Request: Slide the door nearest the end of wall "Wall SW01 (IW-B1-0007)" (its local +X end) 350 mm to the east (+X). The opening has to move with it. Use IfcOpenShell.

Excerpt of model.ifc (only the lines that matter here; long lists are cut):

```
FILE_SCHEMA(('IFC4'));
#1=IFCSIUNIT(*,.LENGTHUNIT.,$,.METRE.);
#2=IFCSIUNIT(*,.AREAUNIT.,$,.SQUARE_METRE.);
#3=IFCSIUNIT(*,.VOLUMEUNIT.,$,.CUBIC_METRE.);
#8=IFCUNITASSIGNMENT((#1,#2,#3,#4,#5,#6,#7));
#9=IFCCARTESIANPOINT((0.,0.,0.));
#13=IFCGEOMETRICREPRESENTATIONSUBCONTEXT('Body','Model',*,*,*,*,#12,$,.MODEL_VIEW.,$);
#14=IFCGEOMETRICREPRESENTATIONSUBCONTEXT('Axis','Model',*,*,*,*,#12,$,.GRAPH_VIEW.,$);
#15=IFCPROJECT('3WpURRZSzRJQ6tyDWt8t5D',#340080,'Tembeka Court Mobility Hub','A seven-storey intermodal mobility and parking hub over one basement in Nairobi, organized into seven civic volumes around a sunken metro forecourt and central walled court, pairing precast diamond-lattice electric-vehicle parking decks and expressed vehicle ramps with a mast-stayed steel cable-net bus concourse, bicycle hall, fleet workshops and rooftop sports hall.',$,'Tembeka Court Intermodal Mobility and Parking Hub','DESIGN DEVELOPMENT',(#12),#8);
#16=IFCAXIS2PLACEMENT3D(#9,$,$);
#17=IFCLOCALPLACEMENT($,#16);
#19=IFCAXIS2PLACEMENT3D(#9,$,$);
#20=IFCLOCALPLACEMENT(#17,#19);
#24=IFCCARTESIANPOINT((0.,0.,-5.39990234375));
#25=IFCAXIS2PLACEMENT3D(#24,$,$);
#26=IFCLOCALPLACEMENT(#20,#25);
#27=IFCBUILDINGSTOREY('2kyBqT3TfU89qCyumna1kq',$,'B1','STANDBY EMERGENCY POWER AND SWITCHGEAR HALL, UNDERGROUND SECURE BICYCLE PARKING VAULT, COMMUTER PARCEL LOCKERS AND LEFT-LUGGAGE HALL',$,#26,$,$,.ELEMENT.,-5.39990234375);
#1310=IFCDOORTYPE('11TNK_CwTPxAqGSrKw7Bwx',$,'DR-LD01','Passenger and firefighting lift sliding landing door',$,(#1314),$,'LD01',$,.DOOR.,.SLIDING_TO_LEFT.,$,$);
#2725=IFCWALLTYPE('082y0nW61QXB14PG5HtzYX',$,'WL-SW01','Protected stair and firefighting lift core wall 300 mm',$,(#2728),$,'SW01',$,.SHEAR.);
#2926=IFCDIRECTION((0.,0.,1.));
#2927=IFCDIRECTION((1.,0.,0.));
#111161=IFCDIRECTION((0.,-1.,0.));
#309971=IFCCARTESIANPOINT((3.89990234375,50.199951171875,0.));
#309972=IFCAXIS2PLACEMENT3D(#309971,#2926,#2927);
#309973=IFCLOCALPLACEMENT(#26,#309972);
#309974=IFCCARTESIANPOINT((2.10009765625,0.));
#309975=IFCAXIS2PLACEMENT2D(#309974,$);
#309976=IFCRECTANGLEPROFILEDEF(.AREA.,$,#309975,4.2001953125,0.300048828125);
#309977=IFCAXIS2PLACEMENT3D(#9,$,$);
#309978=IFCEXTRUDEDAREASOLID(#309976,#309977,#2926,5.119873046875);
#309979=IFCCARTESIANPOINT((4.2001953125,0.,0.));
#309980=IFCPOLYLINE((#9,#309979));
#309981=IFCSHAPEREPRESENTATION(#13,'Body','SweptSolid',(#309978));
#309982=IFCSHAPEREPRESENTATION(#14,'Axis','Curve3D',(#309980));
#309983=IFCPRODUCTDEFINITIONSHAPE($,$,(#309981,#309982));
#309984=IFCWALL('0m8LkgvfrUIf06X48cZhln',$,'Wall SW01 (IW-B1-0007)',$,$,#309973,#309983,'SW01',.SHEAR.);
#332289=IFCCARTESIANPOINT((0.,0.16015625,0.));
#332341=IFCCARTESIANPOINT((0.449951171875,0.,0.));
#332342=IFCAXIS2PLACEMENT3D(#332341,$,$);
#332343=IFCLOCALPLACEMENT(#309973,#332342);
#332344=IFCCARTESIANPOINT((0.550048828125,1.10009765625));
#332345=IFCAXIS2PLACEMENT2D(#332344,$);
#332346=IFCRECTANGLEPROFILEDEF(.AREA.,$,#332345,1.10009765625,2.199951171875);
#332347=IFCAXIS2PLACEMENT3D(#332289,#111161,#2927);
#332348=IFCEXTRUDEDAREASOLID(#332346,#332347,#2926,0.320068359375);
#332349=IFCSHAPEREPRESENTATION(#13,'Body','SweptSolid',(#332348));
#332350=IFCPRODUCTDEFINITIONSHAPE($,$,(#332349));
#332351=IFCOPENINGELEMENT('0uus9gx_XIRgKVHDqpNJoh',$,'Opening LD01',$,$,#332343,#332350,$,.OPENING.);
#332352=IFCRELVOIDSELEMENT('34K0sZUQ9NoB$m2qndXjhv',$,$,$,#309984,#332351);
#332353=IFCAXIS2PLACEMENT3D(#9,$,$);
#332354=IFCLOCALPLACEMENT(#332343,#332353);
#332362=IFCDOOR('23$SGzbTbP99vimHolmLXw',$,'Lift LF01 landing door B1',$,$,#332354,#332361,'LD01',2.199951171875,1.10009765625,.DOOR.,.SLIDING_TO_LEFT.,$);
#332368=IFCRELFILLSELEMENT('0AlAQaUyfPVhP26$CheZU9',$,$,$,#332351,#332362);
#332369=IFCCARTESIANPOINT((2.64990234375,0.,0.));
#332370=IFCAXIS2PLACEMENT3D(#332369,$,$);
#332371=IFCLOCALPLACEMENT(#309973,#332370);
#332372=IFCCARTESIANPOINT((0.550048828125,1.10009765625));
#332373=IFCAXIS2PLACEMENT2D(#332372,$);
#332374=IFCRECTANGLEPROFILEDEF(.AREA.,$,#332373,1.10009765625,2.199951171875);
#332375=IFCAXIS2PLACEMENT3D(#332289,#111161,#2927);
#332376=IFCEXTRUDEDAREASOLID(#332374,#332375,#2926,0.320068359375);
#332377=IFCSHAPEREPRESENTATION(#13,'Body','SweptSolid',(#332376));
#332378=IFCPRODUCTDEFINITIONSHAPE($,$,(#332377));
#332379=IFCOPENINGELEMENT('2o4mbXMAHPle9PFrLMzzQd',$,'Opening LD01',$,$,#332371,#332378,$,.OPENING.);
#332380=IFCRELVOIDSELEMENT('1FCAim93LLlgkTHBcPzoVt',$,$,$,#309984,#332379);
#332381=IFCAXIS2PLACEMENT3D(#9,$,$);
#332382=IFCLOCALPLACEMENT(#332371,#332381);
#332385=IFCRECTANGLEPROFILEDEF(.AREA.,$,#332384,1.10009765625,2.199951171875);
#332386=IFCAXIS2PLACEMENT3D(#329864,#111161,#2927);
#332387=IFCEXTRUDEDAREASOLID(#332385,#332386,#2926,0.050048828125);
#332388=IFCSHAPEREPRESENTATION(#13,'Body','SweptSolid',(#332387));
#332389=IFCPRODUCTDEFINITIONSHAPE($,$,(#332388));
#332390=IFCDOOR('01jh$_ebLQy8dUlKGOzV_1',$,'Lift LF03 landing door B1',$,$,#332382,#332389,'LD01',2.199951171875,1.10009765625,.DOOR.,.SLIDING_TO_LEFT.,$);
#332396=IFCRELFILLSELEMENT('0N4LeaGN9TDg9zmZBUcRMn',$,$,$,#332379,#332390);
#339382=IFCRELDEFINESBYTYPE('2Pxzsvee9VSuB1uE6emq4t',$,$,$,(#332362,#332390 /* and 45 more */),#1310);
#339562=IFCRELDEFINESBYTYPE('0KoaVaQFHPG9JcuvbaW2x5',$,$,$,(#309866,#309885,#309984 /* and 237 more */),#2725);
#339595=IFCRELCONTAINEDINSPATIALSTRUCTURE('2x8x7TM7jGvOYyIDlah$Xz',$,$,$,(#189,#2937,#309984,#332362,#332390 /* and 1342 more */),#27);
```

```python
import ifcopenshell
import ifcopenshell.api.geometry
import ifcopenshell.util.placement
import ifcopenshell.util.unit

model = ifcopenshell.open("model.ifc")
unit_scale = ifcopenshell.util.unit.calculate_unit_scale(model)

door = model.by_guid("01jh$_ebLQy8dUlKGOzV_1")
opening = door.FillsVoids[0].RelatingOpeningElement
wall = opening.VoidsElements[0].RelatingBuildingElement

wall_matrix = ifcopenshell.util.placement.get_local_placement(wall.ObjectPlacement)
shift = wall_matrix[:3, 0] * 0.35 / unit_scale
before = ifcopenshell.util.placement.get_local_placement(door.ObjectPlacement)[:3, 3].copy()

# The door is placed relative to its opening, so it follows when the opening moves.
matrix = ifcopenshell.util.placement.get_local_placement(opening.ObjectPlacement)
matrix[:3, 3] += shift
ifcopenshell.api.geometry.edit_object_placement(
    model, product=opening, matrix=matrix, is_si=False, should_transform_children=True
)

after = ifcopenshell.util.placement.get_local_placement(door.ObjectPlacement)[:3, 3]
print("door moved by", (after - before).round(3) + 0.0)

model.write("model-out.ifc")
```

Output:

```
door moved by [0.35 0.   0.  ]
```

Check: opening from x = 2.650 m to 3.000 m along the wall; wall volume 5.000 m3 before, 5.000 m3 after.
